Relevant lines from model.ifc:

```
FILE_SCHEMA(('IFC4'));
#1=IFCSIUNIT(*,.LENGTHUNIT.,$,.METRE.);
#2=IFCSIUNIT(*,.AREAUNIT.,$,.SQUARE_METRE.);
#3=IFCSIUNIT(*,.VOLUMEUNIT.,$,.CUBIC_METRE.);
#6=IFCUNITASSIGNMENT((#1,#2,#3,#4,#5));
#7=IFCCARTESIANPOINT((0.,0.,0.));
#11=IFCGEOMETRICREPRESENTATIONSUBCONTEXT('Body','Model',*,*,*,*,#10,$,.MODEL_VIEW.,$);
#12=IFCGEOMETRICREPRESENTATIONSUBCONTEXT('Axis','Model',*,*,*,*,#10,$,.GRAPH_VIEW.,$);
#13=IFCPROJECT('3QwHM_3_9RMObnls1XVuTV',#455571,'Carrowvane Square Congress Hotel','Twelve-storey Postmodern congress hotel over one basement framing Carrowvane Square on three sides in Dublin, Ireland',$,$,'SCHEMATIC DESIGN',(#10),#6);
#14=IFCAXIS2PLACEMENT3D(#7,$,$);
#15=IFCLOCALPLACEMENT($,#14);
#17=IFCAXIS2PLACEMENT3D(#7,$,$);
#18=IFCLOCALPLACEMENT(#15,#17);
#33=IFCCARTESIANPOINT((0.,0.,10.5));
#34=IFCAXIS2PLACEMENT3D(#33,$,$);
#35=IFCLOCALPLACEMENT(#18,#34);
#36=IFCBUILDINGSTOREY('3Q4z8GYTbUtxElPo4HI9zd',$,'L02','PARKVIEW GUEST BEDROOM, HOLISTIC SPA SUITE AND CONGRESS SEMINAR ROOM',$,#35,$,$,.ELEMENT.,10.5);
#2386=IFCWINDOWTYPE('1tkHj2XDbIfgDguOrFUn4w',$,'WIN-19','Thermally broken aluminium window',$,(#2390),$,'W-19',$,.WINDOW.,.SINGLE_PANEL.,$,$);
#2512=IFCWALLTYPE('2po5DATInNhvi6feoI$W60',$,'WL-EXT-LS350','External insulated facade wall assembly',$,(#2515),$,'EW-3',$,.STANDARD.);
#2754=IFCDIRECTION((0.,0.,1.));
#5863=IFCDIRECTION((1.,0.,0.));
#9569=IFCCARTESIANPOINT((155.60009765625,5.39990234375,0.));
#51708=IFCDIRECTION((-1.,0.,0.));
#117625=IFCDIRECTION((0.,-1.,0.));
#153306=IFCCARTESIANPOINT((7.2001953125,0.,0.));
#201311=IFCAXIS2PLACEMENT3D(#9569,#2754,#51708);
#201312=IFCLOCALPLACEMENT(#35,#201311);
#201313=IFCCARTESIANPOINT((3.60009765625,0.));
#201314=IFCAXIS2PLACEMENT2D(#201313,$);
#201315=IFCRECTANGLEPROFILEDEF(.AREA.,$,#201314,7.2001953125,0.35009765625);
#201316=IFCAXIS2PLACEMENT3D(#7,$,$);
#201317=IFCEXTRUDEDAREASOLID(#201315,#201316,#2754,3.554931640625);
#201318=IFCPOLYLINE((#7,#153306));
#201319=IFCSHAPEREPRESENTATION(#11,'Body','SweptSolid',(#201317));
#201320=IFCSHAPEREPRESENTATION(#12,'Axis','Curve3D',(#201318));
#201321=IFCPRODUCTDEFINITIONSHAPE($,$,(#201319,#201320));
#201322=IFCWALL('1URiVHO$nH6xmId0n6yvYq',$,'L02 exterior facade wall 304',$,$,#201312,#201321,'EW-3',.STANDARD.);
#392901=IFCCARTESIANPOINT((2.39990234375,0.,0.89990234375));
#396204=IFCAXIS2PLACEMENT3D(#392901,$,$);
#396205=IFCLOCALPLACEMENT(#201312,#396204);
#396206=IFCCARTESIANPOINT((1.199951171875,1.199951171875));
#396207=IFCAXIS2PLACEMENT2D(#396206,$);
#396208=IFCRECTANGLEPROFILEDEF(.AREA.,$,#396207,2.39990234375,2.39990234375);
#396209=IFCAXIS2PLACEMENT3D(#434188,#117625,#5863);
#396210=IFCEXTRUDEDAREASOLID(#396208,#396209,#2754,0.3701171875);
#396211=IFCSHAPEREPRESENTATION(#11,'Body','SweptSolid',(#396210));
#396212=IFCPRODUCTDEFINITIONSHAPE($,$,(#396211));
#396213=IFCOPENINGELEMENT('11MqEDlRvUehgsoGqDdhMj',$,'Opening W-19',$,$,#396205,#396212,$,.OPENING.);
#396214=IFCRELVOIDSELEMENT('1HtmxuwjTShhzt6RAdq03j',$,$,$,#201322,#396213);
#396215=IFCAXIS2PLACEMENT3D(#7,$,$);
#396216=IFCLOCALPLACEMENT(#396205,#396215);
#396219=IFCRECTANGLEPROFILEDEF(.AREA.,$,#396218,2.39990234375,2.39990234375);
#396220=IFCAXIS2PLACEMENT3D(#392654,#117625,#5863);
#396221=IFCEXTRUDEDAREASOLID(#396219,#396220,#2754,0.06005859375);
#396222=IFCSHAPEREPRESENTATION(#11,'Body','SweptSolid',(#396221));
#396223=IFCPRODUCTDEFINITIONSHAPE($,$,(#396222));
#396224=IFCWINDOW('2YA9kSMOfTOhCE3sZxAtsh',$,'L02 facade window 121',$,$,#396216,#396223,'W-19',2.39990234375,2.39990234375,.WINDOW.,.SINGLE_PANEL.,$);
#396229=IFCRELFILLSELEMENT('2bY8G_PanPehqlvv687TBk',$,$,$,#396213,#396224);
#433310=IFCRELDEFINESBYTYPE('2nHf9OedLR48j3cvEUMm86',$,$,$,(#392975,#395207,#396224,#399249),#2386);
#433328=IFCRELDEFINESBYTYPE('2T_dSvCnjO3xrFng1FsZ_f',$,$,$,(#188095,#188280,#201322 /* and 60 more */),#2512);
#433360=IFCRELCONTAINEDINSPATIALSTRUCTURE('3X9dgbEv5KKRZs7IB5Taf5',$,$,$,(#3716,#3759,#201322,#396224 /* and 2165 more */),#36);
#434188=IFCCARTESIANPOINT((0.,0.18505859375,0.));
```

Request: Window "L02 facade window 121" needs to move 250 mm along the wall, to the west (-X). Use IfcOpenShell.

```python
import ifcopenshell
import ifcopenshell.api.geometry
import ifcopenshell.util.placement
import ifcopenshell.util.unit

model = ifcopenshell.open("model.ifc")
unit_scale = ifcopenshell.util.unit.calculate_unit_scale(model)

window = model.by_guid("2YA9kSMOfTOhCE3sZxAtsh")
opening = window.FillsVoids[0].RelatingOpeningElement
wall = opening.VoidsElements[0].RelatingBuildingElement

wall_matrix = ifcopenshell.util.placement.get_local_placement(wall.ObjectPlacement)
shift = wall_matrix[:3, 0] * 0.25 / unit_scale
before = ifcopenshell.util.placement.get_local_placement(window.ObjectPlacement)[:3, 3].copy()

# The window is placed relative to its opening, so it follows when the opening moves.
matrix = ifcopenshell.util.placement.get_local_placement(opening.ObjectPlacement)
matrix[:3, 3] += shift
ifcopenshell.api.geometry.edit_object_placement(
    model, product=opening, matrix=matrix, is_si=False, should_transform_children=True
)

after = ifcopenshell.util.placement.get_local_placement(window.ObjectPlacement)[:3, 3]
print("window moved by", (after - before).round(3) + 0.0)

model.write("model_updated.ifc")
```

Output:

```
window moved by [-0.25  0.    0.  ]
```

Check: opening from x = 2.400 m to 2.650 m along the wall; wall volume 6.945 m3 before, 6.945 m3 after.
